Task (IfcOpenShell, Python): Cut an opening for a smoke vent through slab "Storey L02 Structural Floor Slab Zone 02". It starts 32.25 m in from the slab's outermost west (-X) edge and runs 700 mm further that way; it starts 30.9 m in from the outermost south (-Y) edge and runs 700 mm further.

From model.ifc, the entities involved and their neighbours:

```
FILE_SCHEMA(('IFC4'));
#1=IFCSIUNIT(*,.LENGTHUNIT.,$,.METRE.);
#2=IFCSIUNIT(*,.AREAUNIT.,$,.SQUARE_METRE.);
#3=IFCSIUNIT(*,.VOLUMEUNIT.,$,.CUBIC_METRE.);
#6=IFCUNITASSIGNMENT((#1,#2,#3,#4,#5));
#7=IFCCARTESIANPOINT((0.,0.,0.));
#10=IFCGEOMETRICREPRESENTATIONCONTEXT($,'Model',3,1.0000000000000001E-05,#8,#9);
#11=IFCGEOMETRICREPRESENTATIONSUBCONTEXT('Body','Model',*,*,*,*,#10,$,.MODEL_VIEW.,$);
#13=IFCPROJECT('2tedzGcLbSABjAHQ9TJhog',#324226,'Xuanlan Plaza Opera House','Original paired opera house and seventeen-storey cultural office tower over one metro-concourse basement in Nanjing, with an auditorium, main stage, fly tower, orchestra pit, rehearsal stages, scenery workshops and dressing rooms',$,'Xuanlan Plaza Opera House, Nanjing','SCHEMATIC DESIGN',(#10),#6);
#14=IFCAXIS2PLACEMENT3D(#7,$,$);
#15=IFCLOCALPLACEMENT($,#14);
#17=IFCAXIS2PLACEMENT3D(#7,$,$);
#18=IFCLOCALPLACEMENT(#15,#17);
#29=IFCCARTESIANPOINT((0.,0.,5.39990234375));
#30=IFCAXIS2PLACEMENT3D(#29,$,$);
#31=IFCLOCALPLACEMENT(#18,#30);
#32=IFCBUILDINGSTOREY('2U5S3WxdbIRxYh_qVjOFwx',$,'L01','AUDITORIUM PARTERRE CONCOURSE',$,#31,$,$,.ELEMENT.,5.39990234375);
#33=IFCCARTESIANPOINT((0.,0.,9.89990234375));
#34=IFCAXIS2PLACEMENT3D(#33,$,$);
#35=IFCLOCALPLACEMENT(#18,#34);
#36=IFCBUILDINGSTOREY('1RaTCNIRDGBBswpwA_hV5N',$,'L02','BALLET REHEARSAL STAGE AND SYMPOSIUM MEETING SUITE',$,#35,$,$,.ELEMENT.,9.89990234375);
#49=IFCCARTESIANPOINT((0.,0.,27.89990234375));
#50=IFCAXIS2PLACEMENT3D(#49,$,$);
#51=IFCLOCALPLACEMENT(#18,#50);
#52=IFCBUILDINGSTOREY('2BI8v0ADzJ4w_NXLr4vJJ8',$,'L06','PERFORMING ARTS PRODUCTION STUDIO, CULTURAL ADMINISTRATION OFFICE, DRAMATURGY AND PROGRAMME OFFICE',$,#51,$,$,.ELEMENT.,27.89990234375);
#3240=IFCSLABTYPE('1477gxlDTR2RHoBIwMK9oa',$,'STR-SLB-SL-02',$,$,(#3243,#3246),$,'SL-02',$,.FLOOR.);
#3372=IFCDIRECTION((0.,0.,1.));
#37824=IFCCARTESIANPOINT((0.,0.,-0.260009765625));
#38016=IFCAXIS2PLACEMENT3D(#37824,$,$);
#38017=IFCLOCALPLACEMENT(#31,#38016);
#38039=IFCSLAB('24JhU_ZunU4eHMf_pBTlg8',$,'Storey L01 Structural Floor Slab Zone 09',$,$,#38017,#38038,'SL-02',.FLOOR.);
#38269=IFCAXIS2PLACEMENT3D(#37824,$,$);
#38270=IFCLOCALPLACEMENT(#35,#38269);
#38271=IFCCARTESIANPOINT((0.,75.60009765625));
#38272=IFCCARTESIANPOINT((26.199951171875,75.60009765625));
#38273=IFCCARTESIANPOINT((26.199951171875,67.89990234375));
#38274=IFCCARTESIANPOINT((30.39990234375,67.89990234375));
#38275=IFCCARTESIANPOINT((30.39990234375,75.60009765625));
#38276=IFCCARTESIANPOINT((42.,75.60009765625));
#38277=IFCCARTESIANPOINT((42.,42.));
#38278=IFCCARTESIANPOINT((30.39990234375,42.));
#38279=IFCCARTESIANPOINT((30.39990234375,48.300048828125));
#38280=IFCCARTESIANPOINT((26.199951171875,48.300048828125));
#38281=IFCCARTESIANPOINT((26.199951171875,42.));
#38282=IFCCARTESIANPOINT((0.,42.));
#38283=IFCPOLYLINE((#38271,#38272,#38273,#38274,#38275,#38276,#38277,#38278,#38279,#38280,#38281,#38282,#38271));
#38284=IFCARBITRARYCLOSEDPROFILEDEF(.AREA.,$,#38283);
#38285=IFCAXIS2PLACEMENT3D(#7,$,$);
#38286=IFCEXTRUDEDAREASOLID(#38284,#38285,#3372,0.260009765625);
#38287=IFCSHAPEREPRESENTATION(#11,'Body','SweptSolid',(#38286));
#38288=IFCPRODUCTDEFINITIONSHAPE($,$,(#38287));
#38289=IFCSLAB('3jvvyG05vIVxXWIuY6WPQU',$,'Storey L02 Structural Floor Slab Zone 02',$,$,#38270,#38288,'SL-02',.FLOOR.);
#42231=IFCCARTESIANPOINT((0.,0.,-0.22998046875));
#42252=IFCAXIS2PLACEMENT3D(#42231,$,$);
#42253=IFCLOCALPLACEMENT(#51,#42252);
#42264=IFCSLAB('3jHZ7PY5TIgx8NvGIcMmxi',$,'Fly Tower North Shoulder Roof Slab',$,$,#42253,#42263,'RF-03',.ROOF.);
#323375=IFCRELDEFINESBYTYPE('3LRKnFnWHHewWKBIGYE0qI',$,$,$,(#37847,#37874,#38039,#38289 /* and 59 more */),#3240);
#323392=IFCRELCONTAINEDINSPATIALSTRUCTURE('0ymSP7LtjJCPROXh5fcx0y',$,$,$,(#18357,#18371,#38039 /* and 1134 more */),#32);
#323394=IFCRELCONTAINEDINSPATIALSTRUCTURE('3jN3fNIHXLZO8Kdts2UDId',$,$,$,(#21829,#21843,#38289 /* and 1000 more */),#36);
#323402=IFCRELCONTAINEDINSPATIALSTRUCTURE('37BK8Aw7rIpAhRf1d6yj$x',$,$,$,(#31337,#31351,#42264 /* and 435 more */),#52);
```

```python
import numpy as np
import ifcopenshell
import ifcopenshell.api.feature
import ifcopenshell.api.geometry
import ifcopenshell.api.root
import ifcopenshell.geom
import ifcopenshell.util.placement
import ifcopenshell.util.representation
import ifcopenshell.util.shape
import ifcopenshell.util.unit

model = ifcopenshell.open("model.ifc")
unit_scale = ifcopenshell.util.unit.calculate_unit_scale(model)
settings = ifcopenshell.geom.settings()


def volume(element):
    """Net volume in cubic metres, openings subtracted."""
    shape = ifcopenshell.geom.create_shape(settings, element)
    return ifcopenshell.util.shape.get_volume(shape.geometry)


slab = model.by_id(38289)
before = volume(slab)

# Extent in the slab's own axes, in metres. The edges named are its -X and -Y sides.
slab_shape = ifcopenshell.geom.create_shape(settings, slab)
vertices = ifcopenshell.util.shape.get_vertices(slab_shape.geometry)
x_min, y_min, bottom = vertices.min(axis=0)
top = vertices[:, 2].max()

opening = ifcopenshell.api.root.create_entity(model, ifc_class="IfcOpeningElement", name="Smoke vent opening", predefined_type="OPENING")
context = ifcopenshell.util.representation.get_context(model, "Model", "Body", "MODEL_VIEW")
width, depth = 0.7, 0.7
outline = [(0.0, 0.0), (width, 0.0), (width, depth), (0.0, depth), (0.0, 0.0)]
# Overshoot both faces by 50 mm so the cut is clean.
shape = ifcopenshell.api.geometry.add_slab_representation(
    model, context=context, depth=top - bottom + 0.1, polyline=outline
)
ifcopenshell.api.geometry.assign_representation(model, product=opening, representation=shape)

matrix = ifcopenshell.util.placement.get_local_placement(slab.ObjectPlacement)
matrix[:, 3] = matrix @ np.append(np.array([x_min + 32.25, y_min + 30.9, bottom - 0.05]) / unit_scale, 1.0)
ifcopenshell.api.geometry.edit_object_placement(model, product=opening, matrix=matrix, is_si=False)
ifcopenshell.api.feature.add_feature(model, feature=opening, element=slab)

after = volume(slab)

print(f"slab volume {before:.3f} -> {after:.3f} m3")

model.write("model_rev.ifc")
```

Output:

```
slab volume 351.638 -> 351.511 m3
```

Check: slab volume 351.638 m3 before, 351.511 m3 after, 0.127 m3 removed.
